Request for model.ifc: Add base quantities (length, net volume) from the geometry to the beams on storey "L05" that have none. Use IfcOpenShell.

First a look at what the model holds.

```python
import ifcopenshell
import ifcopenshell.util.element
import ifcopenshell.util.unit

model = ifcopenshell.open("model.ifc")
print(model.schema)
for unit_type in ("LENGTHUNIT", "AREAUNIT", "VOLUMEUNIT"):
    print(unit_type, ifcopenshell.util.unit.calculate_unit_scale(model, unit_type))
storey = next(s for s in model.by_type("IfcBuildingStorey") if s.Name == "L05")
beams = [e for e in ifcopenshell.util.element.get_decomposition(storey) if e.is_a("IfcBeam")]
for e in sorted(beams, key=lambda e: e.id()):
    print(e.id(), e.is_a(), e.Name, list(ifcopenshell.util.element.get_psets(e, qtos_only=True)), sep=" | ")
```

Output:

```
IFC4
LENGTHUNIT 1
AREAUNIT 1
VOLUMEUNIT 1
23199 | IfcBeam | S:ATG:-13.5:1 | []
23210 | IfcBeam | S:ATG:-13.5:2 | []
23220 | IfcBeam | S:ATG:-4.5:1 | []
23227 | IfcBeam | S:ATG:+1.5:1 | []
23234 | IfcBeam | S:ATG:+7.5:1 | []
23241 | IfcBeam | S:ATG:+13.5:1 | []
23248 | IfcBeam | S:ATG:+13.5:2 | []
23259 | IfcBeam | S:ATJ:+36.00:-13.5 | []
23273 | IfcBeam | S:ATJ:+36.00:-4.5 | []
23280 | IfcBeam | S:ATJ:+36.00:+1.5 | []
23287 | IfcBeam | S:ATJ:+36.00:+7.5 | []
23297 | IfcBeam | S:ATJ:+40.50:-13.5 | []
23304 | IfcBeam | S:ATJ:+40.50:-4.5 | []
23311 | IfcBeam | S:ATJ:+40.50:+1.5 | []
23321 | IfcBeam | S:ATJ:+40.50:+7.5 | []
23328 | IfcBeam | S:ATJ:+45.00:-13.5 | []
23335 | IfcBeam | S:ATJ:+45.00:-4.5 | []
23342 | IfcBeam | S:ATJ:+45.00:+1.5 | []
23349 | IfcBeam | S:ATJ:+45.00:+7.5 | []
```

```python
import ifcopenshell
import ifcopenshell.api.pset
import ifcopenshell.geom
import ifcopenshell.util.element
import ifcopenshell.util.shape
import ifcopenshell.util.unit

model = ifcopenshell.open("model.ifc")
unit_scale = ifcopenshell.util.unit.calculate_unit_scale(model)
volume_scale = ifcopenshell.util.unit.calculate_unit_scale(model, "VOLUMEUNIT")
settings = ifcopenshell.geom.settings()

storey = next(s for s in model.by_type("IfcBuildingStorey") if s.Name == "L05")
beams = [e for e in ifcopenshell.util.element.get_decomposition(storey) if e.is_a("IfcBeam")]

for e in sorted(beams, key=lambda e: e.id()):
    if ifcopenshell.util.element.get_psets(e, qtos_only=True, should_inherit=False):
        continue
    # Geometry comes back in metres, in the element's own axes.
    shape = ifcopenshell.geom.create_shape(settings, e)
    values = {
        "Length": ifcopenshell.util.shape.get_max_xyz(shape.geometry) / unit_scale,
        "NetVolume": ifcopenshell.util.shape.get_volume(shape.geometry) / volume_scale,
    }
    qto = ifcopenshell.api.pset.add_qto(model, product=e, name="Qto_BeamBaseQuantities")
    ifcopenshell.api.pset.edit_qto(model, qto=qto, properties=values)
    print(e.id(), {k: round(v, 3) for k, v in values.items()})

model.write("model_v2.ifc")
```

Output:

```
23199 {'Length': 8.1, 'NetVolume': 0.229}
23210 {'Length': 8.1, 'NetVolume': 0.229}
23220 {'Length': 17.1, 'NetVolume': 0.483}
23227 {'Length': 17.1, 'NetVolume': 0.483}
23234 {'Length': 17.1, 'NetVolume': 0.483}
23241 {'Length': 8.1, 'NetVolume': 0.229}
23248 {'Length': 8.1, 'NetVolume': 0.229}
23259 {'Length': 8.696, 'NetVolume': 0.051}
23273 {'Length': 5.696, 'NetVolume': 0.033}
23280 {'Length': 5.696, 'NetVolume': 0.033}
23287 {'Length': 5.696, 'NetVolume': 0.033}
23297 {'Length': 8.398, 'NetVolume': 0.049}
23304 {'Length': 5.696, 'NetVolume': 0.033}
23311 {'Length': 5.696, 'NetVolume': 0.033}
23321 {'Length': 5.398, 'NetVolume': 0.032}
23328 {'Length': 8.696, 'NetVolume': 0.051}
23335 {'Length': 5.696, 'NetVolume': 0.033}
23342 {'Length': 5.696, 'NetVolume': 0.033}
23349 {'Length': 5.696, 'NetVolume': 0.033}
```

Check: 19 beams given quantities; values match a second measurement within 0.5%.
